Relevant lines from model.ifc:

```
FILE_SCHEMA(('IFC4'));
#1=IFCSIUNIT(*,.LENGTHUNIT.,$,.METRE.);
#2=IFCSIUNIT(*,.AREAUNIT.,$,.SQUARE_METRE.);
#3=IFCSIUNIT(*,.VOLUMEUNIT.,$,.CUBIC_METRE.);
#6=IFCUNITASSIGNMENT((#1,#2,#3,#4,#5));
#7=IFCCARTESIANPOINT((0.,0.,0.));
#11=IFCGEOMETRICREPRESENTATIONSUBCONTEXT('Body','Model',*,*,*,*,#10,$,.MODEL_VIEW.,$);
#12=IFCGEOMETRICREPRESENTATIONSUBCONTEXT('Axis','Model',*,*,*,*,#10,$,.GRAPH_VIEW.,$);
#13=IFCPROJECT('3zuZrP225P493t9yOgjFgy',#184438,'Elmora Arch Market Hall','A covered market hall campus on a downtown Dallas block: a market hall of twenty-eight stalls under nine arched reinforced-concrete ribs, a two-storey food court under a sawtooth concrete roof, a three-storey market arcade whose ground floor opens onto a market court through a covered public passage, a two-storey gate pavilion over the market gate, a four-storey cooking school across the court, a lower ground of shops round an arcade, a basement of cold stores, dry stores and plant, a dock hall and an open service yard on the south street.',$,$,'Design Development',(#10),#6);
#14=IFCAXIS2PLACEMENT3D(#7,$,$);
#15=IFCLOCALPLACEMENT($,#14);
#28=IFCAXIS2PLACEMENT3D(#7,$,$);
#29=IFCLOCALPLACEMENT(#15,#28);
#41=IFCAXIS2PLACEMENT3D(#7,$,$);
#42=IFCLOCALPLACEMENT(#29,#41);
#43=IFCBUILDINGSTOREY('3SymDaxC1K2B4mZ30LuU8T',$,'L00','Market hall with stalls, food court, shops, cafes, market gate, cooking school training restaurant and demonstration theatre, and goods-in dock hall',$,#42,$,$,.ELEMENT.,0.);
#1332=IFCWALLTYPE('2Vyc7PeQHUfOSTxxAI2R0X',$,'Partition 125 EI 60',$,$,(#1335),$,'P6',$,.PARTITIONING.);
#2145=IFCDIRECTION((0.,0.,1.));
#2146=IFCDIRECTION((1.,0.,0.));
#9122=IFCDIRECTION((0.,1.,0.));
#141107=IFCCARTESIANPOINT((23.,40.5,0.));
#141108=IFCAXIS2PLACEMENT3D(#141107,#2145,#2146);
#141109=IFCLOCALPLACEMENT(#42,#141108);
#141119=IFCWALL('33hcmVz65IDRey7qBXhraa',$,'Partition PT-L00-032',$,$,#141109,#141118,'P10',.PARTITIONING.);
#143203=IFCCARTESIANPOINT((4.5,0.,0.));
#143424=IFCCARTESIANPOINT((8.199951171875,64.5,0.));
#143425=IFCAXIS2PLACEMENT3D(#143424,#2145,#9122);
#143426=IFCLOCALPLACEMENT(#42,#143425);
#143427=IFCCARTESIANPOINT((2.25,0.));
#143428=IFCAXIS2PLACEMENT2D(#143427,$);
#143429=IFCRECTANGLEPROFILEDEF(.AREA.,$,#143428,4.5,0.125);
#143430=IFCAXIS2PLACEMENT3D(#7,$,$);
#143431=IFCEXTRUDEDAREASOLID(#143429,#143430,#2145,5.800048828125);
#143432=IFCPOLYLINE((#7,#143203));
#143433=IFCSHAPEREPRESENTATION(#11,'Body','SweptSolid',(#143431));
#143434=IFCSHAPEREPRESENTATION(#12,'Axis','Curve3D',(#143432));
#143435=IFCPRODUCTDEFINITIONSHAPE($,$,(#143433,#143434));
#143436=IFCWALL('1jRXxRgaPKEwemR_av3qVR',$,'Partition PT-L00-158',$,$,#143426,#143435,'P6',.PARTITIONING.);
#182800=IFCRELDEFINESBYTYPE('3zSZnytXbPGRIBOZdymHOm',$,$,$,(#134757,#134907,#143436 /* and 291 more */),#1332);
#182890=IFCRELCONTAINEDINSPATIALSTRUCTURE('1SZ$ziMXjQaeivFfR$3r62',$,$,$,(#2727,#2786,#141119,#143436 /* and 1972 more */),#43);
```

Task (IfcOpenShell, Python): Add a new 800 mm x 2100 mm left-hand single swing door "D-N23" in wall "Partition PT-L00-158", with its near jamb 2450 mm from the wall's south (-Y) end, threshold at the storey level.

```python
import numpy as np
import ifcopenshell
import ifcopenshell.api.feature
import ifcopenshell.api.geometry
import ifcopenshell.api.root
import ifcopenshell.api.spatial
import ifcopenshell.geom
import ifcopenshell.util.element
import ifcopenshell.util.placement
import ifcopenshell.util.representation
import ifcopenshell.util.shape
import ifcopenshell.util.unit

model = ifcopenshell.open("model.ifc")
unit_scale = ifcopenshell.util.unit.calculate_unit_scale(model)
settings = ifcopenshell.geom.settings()


def volume(element):
    """Net volume in cubic metres, openings subtracted."""
    shape = ifcopenshell.geom.create_shape(settings, element)
    return ifcopenshell.util.shape.get_volume(shape.geometry)


wall = model.by_guid("1jRXxRgaPKEwemR_av3qVR")
storey = ifcopenshell.util.element.get_container(wall, ifc_class="IfcBuildingStorey")
context = ifcopenshell.util.representation.get_context(model, "Model", "Body", "MODEL_VIEW")
before = volume(wall)

width, height, from_end, sill = 0.8, 2.1, 2.45, 0.0  # metres

# The wall runs along its own X axis, and the end named is its -X end.
wall_shape = ifcopenshell.geom.create_shape(settings, wall)
x, y, z = ifcopenshell.util.shape.get_vertices(wall_shape.geometry).T
start = x.min() + from_end
face, thickness = float(y.min()), float(y.max() - y.min())
wall_matrix = ifcopenshell.util.placement.get_local_placement(wall.ObjectPlacement)
level = ifcopenshell.util.placement.get_local_placement(storey.ObjectPlacement)[2, 3]


def in_wall(x, y):
    """Placement at x, y metres in the wall's axes, at sill height."""
    matrix = wall_matrix.copy()
    matrix[:, 3] = wall_matrix @ np.array([x / unit_scale, y / unit_scale, 0.0, 1.0])
    matrix[2, 3] = level + sill / unit_scale
    return matrix


# Opening: a box that overshoots both wall faces by 50 mm.
opening = ifcopenshell.api.root.create_entity(model, ifc_class="IfcOpeningElement", predefined_type="OPENING")
box = ifcopenshell.api.geometry.add_wall_representation(
    model, context=context, length=width, height=height, thickness=thickness + 0.1
)
ifcopenshell.api.geometry.assign_representation(model, product=opening, representation=box)
ifcopenshell.api.geometry.edit_object_placement(model, product=opening, matrix=in_wall(start, face - 0.05), is_si=False)
ifcopenshell.api.feature.add_feature(model, feature=opening, element=wall)

door = ifcopenshell.api.root.create_entity(model, ifc_class="IfcDoor", name="D-N23", predefined_type="DOOR")
door.OverallWidth, door.OverallHeight = width / unit_scale, height / unit_scale
door.OperationType = "SINGLE_SWING_LEFT"
body = ifcopenshell.api.geometry.add_door_representation(
    model,
    context=context,
    overall_width=door.OverallWidth,
    overall_height=door.OverallHeight,
    operation_type="SINGLE_SWING_LEFT",
    lining_properties={"LiningDepth": thickness / unit_scale, "ThresholdDepth": thickness / unit_scale},
)
ifcopenshell.api.geometry.assign_representation(model, product=door, representation=body)
ifcopenshell.api.spatial.assign_container(model, products=[door], relating_structure=storey)
ifcopenshell.api.feature.add_filling(model, opening=opening, element=door)

# The lining spans the wall, so the door starts at the wall face.
ifcopenshell.api.geometry.edit_object_placement(model, product=door, matrix=in_wall(start, face), is_si=False)

after = volume(wall)

print(f"wall volume {before:.3f} -> {after:.3f} m3")

model.write("model_rev.ifc")
```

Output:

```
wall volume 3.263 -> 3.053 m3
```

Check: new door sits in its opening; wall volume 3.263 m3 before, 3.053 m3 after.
